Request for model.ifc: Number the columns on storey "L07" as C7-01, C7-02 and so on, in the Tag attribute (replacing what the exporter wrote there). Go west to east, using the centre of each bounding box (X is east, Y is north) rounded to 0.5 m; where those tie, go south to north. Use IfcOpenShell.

First a look at what the model holds.

```python
import ifcopenshell
import ifcopenshell.util.element
import ifcopenshell.util.placement

model = ifcopenshell.open("model.ifc")
print(model.schema)
storey = next(s for s in model.by_type("IfcBuildingStorey") if s.Name == "L07")
columns = [e for e in ifcopenshell.util.element.get_decomposition(storey) if e.is_a("IfcColumn")]
for e in sorted(columns, key=lambda e: e.id()):
    origin = ifcopenshell.util.placement.get_local_placement(e.ObjectPlacement)[:3, 3]
    print(e.id(), e.Tag, e.Name, origin.round(2) + 0.0, sep=" | ")
```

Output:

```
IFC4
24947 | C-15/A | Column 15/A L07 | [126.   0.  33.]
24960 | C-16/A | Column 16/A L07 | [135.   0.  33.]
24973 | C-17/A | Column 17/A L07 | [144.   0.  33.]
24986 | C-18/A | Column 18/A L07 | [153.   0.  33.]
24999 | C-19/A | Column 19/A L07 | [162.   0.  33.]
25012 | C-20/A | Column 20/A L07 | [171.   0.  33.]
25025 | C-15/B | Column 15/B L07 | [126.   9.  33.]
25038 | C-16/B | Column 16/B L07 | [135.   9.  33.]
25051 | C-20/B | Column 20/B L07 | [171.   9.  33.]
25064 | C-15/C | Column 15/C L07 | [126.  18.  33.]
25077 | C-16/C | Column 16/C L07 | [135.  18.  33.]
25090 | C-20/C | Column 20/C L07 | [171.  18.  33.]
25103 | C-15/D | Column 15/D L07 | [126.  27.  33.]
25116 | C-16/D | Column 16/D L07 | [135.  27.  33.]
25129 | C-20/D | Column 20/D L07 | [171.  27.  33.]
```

```python
import ifcopenshell
import ifcopenshell.geom
import ifcopenshell.util.element
import ifcopenshell.util.shape

model = ifcopenshell.open("model.ifc")
settings = ifcopenshell.geom.settings()
settings.set("use-world-coords", True)


def centre(element):
    shape = ifcopenshell.geom.create_shape(settings, element)
    return ifcopenshell.util.shape.get_bbox_centroid(shape.geometry)


storey = next(s for s in model.by_type("IfcBuildingStorey") if s.Name == "L07")
columns = [e for e in ifcopenshell.util.element.get_decomposition(storey) if e.is_a("IfcColumn")]

# Insertion points can sit at a corner or the storey origin, so sort by the geometry (in metres).
centres = {e: centre(e) for e in columns}
columns.sort(key=lambda e: (round(centres[e][0] / 0.5), centres[e][1]))

for i, e in enumerate(columns, start=1):
    number = f"C7-{i:02d}"
    e.Tag = number
    print(e.id(), number)

model.write("model_rev.ifc")
```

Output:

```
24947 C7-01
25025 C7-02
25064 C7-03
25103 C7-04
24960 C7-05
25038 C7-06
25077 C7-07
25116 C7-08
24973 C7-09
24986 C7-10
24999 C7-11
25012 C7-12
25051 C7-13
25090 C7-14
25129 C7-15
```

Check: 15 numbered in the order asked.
